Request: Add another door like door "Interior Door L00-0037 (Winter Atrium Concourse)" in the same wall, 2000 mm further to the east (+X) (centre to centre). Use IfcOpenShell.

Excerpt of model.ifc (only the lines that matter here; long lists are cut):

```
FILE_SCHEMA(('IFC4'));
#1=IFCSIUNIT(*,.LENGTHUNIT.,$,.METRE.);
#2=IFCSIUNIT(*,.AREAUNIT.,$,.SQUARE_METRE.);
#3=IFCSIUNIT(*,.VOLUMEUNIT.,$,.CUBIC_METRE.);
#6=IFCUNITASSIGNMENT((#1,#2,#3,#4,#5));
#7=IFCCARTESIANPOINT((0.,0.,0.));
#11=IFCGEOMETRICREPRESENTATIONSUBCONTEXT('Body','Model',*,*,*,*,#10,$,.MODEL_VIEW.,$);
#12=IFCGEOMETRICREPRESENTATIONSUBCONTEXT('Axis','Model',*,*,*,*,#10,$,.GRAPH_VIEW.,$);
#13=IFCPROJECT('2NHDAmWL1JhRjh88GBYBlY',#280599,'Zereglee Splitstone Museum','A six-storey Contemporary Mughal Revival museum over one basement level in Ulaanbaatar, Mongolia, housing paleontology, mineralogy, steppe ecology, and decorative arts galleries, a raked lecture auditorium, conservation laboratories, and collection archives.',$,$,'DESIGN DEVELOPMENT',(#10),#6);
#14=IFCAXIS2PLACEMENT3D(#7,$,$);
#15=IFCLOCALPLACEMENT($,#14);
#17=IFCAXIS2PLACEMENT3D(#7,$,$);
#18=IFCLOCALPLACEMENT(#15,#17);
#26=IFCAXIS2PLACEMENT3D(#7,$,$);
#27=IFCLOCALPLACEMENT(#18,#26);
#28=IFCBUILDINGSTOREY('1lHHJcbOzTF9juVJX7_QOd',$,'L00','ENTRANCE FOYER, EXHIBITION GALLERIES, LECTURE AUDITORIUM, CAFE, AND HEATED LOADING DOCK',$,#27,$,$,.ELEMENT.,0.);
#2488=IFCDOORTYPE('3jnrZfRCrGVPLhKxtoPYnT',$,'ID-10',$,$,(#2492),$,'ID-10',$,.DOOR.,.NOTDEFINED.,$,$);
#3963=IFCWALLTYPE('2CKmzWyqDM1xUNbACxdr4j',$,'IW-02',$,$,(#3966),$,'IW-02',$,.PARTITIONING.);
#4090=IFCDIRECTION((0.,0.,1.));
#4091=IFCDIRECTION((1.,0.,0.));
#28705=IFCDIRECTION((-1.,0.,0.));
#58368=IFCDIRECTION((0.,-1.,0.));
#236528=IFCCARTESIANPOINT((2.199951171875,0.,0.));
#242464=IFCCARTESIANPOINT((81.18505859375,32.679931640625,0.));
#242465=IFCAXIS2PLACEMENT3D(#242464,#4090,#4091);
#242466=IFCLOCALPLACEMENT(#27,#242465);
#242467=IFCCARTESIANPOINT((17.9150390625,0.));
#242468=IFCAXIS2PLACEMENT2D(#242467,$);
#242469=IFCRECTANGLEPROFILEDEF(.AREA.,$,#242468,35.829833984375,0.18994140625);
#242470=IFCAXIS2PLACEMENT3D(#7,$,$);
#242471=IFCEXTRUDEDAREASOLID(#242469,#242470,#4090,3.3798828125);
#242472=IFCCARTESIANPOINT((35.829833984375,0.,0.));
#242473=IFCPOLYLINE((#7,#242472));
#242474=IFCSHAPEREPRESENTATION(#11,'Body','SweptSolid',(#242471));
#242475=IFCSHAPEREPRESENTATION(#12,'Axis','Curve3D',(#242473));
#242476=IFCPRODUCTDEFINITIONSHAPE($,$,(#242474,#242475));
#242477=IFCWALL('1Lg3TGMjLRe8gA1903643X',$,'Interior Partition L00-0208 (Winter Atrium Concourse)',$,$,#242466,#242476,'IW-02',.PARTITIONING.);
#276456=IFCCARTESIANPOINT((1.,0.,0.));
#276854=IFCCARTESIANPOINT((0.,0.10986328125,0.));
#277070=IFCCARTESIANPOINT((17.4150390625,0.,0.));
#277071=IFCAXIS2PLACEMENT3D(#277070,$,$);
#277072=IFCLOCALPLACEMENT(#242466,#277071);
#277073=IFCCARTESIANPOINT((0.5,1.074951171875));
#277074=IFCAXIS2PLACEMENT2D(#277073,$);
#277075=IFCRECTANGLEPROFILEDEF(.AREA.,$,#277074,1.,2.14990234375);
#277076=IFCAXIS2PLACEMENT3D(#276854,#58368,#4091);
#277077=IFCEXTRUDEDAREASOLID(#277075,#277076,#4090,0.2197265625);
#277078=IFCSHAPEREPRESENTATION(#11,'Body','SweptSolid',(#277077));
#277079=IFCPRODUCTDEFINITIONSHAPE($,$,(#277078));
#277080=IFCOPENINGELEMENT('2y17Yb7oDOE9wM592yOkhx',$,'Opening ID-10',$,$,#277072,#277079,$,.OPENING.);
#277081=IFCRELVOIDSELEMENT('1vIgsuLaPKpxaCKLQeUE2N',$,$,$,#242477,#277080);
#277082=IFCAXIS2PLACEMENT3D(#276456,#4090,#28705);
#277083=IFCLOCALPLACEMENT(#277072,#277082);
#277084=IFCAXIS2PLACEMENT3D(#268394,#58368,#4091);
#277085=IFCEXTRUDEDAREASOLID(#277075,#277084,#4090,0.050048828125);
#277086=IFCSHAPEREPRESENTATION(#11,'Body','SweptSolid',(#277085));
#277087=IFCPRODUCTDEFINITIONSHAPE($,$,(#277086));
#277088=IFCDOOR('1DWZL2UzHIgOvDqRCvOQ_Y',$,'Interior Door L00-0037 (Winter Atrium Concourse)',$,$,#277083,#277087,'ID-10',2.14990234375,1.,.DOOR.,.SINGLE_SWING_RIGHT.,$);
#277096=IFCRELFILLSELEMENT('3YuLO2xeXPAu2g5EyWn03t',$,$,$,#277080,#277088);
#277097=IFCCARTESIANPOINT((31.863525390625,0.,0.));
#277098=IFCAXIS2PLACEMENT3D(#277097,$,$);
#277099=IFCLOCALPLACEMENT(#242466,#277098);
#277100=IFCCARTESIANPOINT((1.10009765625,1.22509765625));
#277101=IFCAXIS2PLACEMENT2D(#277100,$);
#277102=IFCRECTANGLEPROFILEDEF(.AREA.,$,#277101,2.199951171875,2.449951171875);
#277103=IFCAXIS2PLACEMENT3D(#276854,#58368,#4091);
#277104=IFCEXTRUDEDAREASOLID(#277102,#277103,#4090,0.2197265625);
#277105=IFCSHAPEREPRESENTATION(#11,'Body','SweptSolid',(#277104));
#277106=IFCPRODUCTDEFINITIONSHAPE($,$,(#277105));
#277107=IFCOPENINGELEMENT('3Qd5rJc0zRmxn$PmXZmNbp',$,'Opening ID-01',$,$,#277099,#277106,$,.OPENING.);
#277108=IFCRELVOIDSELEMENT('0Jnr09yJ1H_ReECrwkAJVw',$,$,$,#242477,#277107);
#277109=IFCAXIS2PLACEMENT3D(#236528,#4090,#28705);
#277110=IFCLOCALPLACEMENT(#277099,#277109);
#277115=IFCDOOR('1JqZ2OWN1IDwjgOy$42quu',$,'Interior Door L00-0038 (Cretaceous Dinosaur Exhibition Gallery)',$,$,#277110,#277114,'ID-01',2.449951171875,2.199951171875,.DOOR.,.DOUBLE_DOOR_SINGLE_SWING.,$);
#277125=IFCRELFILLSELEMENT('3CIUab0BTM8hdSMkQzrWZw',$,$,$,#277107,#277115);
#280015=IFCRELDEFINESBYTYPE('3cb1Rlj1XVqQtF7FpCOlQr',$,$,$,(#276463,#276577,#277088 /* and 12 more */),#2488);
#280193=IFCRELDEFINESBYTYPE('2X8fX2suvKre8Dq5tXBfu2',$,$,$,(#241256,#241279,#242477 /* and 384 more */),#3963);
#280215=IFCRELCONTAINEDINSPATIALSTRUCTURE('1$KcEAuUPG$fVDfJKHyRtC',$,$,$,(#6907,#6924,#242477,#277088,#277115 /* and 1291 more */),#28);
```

```python
import ifcopenshell
import ifcopenshell.api.feature
import ifcopenshell.api.geometry
import ifcopenshell.api.root
import ifcopenshell.geom
import ifcopenshell.util.element
import ifcopenshell.util.placement
import ifcopenshell.util.shape
import ifcopenshell.util.unit

model = ifcopenshell.open("model.ifc")
unit_scale = ifcopenshell.util.unit.calculate_unit_scale(model)
settings = ifcopenshell.geom.settings()


def volume(element):
    """Net volume in cubic metres, openings subtracted."""
    shape = ifcopenshell.geom.create_shape(settings, element)
    return ifcopenshell.util.shape.get_volume(shape.geometry)


door = model.by_id(277088)
opening = door.FillsVoids[0].RelatingOpeningElement
wall = opening.VoidsElements[0].RelatingBuildingElement
before = volume(wall)
shift = ifcopenshell.util.placement.get_local_placement(wall.ObjectPlacement)[:3, 0] * 2 / unit_scale

# copy_class copies the void relationship, type, container and properties, but no geometry.
new_opening = ifcopenshell.api.root.copy_class(model, product=opening)
new_opening.Representation = ifcopenshell.util.element.copy_deep(
    model, opening.Representation, exclude=["IfcGeometricRepresentationContext", "IfcRepresentationMap"]
)
new_door = ifcopenshell.api.root.copy_class(model, product=door)
new_door.Representation = ifcopenshell.util.element.copy_deep(
    model, door.Representation, exclude=["IfcGeometricRepresentationContext", "IfcRepresentationMap"]
)
new_door.Tag = None
ifcopenshell.api.feature.add_filling(model, opening=new_opening, element=new_door)

for old, new in ((opening, new_opening), (door, new_door)):
    matrix = ifcopenshell.util.placement.get_local_placement(old.ObjectPlacement)
    matrix[:3, 3] += shift
    ifcopenshell.api.geometry.edit_object_placement(model, product=new, matrix=matrix, is_si=False)

after = volume(wall)

print(f"wall volume {before:.3f} -> {after:.3f} m3")

model.write("model_updated.ifc")
```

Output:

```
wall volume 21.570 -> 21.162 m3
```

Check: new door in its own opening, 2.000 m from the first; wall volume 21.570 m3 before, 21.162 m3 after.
